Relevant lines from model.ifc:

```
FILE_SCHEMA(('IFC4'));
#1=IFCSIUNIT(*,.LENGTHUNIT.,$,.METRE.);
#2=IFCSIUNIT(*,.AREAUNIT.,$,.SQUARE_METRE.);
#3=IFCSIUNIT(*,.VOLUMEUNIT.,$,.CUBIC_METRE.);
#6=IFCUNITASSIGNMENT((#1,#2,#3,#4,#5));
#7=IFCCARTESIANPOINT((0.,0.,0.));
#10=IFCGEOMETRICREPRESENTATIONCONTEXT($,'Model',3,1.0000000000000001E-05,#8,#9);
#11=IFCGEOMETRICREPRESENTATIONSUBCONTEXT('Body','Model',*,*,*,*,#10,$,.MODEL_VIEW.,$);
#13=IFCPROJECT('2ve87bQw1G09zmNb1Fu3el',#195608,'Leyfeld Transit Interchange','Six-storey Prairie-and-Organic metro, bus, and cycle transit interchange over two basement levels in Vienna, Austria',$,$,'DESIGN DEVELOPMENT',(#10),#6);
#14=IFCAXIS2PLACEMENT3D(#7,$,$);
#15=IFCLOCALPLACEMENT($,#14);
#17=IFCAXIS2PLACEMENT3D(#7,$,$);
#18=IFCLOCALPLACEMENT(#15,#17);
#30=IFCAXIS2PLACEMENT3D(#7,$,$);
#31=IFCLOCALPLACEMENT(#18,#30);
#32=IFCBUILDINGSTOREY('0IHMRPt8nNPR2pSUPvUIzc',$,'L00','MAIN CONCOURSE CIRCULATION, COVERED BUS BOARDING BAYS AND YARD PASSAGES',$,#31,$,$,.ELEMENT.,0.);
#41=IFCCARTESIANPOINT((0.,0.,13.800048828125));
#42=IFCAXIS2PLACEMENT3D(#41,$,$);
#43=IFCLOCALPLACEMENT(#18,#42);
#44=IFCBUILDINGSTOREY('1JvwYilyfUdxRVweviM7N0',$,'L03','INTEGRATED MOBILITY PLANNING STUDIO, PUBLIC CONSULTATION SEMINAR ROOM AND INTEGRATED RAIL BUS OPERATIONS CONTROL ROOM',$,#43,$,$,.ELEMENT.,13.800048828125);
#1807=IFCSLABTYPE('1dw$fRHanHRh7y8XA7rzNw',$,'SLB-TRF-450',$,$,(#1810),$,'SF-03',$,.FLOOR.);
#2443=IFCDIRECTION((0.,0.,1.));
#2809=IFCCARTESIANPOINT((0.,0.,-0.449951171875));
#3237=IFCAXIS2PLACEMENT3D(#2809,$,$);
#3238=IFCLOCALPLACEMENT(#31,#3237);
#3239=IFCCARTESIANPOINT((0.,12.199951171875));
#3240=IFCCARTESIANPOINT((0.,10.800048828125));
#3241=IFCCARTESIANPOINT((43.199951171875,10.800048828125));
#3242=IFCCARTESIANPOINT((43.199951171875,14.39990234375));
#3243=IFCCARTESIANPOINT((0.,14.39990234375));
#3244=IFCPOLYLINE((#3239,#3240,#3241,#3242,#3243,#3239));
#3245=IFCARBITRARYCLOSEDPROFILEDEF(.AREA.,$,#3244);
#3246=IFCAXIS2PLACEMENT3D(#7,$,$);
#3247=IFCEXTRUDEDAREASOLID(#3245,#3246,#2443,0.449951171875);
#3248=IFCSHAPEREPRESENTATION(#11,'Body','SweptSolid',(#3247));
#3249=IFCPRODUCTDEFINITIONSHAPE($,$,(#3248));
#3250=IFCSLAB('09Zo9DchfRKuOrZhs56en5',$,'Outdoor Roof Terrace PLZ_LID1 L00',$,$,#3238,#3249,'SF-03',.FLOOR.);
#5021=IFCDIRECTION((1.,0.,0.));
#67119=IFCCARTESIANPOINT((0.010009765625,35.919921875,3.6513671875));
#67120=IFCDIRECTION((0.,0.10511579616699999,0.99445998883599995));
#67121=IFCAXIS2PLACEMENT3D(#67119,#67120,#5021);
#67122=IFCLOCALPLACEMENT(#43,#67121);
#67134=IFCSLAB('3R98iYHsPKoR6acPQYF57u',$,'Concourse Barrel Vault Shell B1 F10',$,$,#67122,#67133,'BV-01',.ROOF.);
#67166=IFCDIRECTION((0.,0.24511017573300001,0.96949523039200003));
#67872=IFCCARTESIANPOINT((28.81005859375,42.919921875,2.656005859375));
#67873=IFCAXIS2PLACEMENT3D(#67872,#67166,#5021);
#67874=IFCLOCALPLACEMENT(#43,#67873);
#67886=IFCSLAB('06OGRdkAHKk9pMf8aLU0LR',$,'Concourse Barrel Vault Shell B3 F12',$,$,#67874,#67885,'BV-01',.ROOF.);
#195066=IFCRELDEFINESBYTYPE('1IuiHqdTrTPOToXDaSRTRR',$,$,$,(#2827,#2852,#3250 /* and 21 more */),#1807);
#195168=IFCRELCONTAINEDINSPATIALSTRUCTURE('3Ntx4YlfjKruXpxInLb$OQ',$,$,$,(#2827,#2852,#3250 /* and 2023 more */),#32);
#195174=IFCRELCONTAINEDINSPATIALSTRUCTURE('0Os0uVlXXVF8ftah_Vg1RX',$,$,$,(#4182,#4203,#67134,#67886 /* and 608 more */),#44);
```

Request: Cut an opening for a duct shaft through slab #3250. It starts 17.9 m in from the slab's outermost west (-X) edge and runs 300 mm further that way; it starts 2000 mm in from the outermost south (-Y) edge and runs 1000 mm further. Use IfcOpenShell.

```python
import numpy as np
import ifcopenshell
import ifcopenshell.api.feature
import ifcopenshell.api.geometry
import ifcopenshell.api.root
import ifcopenshell.geom
import ifcopenshell.util.placement
import ifcopenshell.util.representation
import ifcopenshell.util.shape
import ifcopenshell.util.unit

model = ifcopenshell.open("model.ifc")
unit_scale = ifcopenshell.util.unit.calculate_unit_scale(model)
settings = ifcopenshell.geom.settings()


def volume(element):
    """Net volume in cubic metres, openings subtracted."""
    shape = ifcopenshell.geom.create_shape(settings, element)
    return ifcopenshell.util.shape.get_volume(shape.geometry)


slab = model.by_guid("09Zo9DchfRKuOrZhs56en5")
before = volume(slab)

# Extent in the slab's own axes, in metres. The edges named are its -X and -Y sides.
slab_shape = ifcopenshell.geom.create_shape(settings, slab)
vertices = ifcopenshell.util.shape.get_vertices(slab_shape.geometry)
x_min, y_min, bottom = vertices.min(axis=0)
top = vertices[:, 2].max()

opening = ifcopenshell.api.root.create_entity(model, ifc_class="IfcOpeningElement", name="Duct shaft opening", predefined_type="OPENING")
context = ifcopenshell.util.representation.get_context(model, "Model", "Body", "MODEL_VIEW")
width, depth = 0.3, 1
outline = [(0.0, 0.0), (width, 0.0), (width, depth), (0.0, depth), (0.0, 0.0)]
# Overshoot both faces by 50 mm so the cut is clean.
shape = ifcopenshell.api.geometry.add_slab_representation(
    model, context=context, depth=top - bottom + 0.1, polyline=outline
)
ifcopenshell.api.geometry.assign_representation(model, product=opening, representation=shape)

matrix = ifcopenshell.util.placement.get_local_placement(slab.ObjectPlacement)
matrix[:, 3] = matrix @ np.append(np.array([x_min + 17.9, y_min + 2, bottom - 0.05]) / unit_scale, 1.0)
ifcopenshell.api.geometry.edit_object_placement(model, product=opening, matrix=matrix, is_si=False)
ifcopenshell.api.feature.add_feature(model, feature=opening, element=slab)

after = volume(slab)

print(f"slab volume {before:.3f} -> {after:.3f} m3")

model.write("model_updated.ifc")
```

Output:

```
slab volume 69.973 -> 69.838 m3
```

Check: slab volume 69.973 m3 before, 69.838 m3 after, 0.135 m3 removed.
